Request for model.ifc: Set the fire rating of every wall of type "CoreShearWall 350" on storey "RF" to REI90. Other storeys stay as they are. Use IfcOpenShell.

First a look at what the model holds.

```python
import ifcopenshell
import ifcopenshell.util.element

model = ifcopenshell.open("model.ifc")
print(model.schema)
storey = next(s for s in model.by_type("IfcBuildingStorey") if s.Name == "RF")
walls = [e for e in ifcopenshell.util.element.get_decomposition(storey) if e.is_a("IfcWall")]
seen = {}
for e in walls:
    element_type = ifcopenshell.util.element.get_type(e)
    key = (element_type.Name if element_type != e and element_type else None, ifcopenshell.util.element.get_pset(e, "Pset_WallCommon", "FireRating"))
    seen[key] = seen.get(key, 0) + 1
for (name, value), count in sorted(seen.items(), key=str):
    print(count, "x", name, "|", value)
```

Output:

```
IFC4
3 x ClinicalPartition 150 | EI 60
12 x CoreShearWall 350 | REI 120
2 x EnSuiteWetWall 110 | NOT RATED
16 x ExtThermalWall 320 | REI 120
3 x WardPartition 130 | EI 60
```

```python
import ifcopenshell
import ifcopenshell.api.pset
import ifcopenshell.util.element

model = ifcopenshell.open("model.ifc")

storey = next(s for s in model.by_type("IfcBuildingStorey") if s.Name == "RF")
walls = [e for e in ifcopenshell.util.element.get_decomposition(storey) if e.is_a("IfcWall")]

count = 0
for e in walls:
    element_type = ifcopenshell.util.element.get_type(e)
    if element_type in (None, e) or element_type.Name != "CoreShearWall 350":
        continue
    # add_pset returns the element's existing set when there is one.
    pset = ifcopenshell.api.pset.add_pset(model, product=e, name="Pset_WallCommon")
    ifcopenshell.api.pset.edit_pset(model, pset=pset, properties={"FireRating": "REI90"})
    count += 1

print(count, "walls updated")

model.write("model_updated.ifc")
```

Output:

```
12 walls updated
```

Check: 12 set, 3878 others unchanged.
